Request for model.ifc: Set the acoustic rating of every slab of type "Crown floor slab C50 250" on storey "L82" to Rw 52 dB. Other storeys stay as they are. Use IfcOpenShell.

First a look at what the model holds.

```python
import ifcopenshell
import ifcopenshell.util.element

model = ifcopenshell.open("model.ifc")
print(model.schema)
storey = next(s for s in model.by_type("IfcBuildingStorey") if s.Name == "L82")
slabs = [e for e in ifcopenshell.util.element.get_decomposition(storey) if e.is_a("IfcSlab")]
seen = {}
for e in slabs:
    element_type = ifcopenshell.util.element.get_type(e)
    key = (element_type.Name if element_type != e and element_type else None, ifcopenshell.util.element.get_pset(e, "Pset_SlabCommon", "AcousticRating"))
    seen[key] = seen.get(key, 0) + 1
for (name, value), count in sorted(seen.items(), key=str):
    print(count, "x", name, "|", value)
```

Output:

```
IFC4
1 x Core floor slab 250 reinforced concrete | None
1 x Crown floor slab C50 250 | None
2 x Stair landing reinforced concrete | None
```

```python
import ifcopenshell
import ifcopenshell.api.pset
import ifcopenshell.util.element

model = ifcopenshell.open("model.ifc")

storey = next(s for s in model.by_type("IfcBuildingStorey") if s.Name == "L82")
slabs = [e for e in ifcopenshell.util.element.get_decomposition(storey) if e.is_a("IfcSlab")]

count = 0
for e in slabs:
    element_type = ifcopenshell.util.element.get_type(e)
    if element_type in (None, e) or element_type.Name != "Crown floor slab C50 250":
        continue
    found = ifcopenshell.util.element.get_pset(e, "Pset_SlabCommon", should_inherit=False)
    if found:
        pset = model.by_id(found["id"])
        if len(ifcopenshell.util.element.get_elements_by_pset(pset)) > 1:
            pset = ifcopenshell.api.pset.unshare_pset(model, products=[e], pset=pset)[0]
    else:
        pset = ifcopenshell.api.pset.add_pset(model, product=e, name="Pset_SlabCommon")
    ifcopenshell.api.pset.edit_pset(model, pset=pset, properties={"AcousticRating": "Rw 52 dB"})
    count += 1

print(count, "slabs updated")

model.write("model_v2.ifc")
```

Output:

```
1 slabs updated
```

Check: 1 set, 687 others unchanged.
